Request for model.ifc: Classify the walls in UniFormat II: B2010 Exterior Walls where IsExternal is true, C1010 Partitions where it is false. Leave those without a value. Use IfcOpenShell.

First a look at what the model holds.

```python
import ifcopenshell
import ifcopenshell.util.element

model = ifcopenshell.open("model.ifc")
print(model.schema)
print("classifications:", [c.Name for c in model.by_type("IfcClassification")])
values = [ifcopenshell.util.element.get_pset(e, "Pset_WallCommon", "IsExternal") for e in model.by_type("IfcWall")]
for value in (True, False, None):
    print("IsExternal", value, values.count(value))
```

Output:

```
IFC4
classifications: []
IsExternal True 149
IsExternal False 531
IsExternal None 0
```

```python
import ifcopenshell
import ifcopenshell.api.classification
import ifcopenshell.util.element

model = ifcopenshell.open("model.ifc")

system = ifcopenshell.api.classification.add_classification(model, classification="UniFormat II")

walls = model.by_type("IfcWall")
external = {e: ifcopenshell.util.element.get_pset(e, "Pset_WallCommon", "IsExternal") for e in walls}
for flag, code, name in ((True, "B2010", "Exterior Walls"), (False, "C1010", "Partitions")):
    products = [e for e in walls if external[e] is flag]
    ifcopenshell.api.classification.add_reference(
        model, products=products, classification=system, identification=code, name=name
    )
    print(code, len(products))

model.write("model_v2.ifc")
```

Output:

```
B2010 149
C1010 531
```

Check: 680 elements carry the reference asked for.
